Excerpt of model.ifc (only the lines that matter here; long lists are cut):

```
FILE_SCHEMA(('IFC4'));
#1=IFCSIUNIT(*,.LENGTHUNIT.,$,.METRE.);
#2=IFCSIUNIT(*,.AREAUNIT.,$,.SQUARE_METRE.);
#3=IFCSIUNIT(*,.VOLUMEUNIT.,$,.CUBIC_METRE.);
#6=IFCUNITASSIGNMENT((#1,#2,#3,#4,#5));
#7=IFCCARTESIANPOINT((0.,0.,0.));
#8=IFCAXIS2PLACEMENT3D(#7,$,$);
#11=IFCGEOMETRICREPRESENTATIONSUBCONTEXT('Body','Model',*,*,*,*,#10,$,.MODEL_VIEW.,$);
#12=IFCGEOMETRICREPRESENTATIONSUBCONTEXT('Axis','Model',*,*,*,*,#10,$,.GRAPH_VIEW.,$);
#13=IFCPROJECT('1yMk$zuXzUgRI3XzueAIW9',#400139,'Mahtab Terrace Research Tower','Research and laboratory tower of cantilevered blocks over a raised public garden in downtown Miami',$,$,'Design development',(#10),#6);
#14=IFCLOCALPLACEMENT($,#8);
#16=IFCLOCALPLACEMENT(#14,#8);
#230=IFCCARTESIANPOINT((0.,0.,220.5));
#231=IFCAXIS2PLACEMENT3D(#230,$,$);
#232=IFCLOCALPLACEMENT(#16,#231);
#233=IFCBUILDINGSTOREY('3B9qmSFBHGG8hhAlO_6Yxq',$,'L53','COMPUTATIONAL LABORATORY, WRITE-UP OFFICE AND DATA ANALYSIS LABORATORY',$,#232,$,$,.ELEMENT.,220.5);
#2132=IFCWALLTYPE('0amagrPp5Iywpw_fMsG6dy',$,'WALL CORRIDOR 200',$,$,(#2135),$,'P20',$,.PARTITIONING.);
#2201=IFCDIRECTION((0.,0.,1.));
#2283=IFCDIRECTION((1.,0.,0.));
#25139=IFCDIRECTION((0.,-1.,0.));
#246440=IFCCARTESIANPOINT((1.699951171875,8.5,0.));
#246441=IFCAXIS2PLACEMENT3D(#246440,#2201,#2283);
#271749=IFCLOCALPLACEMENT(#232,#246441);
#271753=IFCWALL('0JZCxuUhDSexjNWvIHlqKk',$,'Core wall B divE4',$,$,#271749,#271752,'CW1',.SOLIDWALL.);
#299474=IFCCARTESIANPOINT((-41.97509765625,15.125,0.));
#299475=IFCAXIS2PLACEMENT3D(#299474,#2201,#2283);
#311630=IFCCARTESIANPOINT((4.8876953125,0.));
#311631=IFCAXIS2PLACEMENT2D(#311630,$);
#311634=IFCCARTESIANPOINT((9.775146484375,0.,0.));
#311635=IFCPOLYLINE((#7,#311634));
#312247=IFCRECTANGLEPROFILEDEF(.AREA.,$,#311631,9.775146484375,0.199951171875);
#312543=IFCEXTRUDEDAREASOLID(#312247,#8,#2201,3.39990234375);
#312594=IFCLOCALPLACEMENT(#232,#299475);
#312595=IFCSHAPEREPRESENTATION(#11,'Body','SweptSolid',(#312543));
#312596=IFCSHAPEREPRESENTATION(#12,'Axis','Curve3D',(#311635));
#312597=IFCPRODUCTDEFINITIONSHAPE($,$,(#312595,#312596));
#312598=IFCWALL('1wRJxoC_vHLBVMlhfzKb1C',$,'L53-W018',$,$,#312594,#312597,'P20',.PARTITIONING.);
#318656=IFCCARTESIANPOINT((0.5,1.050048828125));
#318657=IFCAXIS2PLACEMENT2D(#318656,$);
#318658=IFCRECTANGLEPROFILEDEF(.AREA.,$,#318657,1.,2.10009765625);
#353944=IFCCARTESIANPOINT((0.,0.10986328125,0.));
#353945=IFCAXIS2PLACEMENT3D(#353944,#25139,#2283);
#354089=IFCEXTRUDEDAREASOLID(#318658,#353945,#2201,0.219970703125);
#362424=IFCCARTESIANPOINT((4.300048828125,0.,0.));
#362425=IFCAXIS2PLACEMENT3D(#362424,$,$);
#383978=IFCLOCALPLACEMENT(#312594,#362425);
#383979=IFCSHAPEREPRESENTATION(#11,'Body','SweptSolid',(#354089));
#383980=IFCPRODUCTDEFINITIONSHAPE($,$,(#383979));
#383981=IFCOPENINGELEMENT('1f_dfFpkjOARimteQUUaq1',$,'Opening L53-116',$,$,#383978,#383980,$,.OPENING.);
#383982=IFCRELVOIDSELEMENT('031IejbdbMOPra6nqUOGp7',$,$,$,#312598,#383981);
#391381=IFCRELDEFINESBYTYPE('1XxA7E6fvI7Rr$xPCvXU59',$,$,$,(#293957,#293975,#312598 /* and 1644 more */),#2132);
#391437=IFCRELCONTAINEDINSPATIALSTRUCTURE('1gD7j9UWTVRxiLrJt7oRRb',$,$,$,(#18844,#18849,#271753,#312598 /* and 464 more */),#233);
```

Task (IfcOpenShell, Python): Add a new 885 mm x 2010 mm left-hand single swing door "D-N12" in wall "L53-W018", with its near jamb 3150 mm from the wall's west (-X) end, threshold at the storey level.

```python
import numpy as np
import ifcopenshell
import ifcopenshell.api.feature
import ifcopenshell.api.geometry
import ifcopenshell.api.root
import ifcopenshell.api.spatial
import ifcopenshell.geom
import ifcopenshell.util.element
import ifcopenshell.util.placement
import ifcopenshell.util.representation
import ifcopenshell.util.shape
import ifcopenshell.util.unit

model = ifcopenshell.open("model.ifc")
unit_scale = ifcopenshell.util.unit.calculate_unit_scale(model)
settings = ifcopenshell.geom.settings()


def volume(element):
    """Net volume in cubic metres, openings subtracted."""
    shape = ifcopenshell.geom.create_shape(settings, element)
    return ifcopenshell.util.shape.get_volume(shape.geometry)


wall = model.by_guid("1wRJxoC_vHLBVMlhfzKb1C")
storey = ifcopenshell.util.element.get_container(wall, ifc_class="IfcBuildingStorey")
context = ifcopenshell.util.representation.get_context(model, "Model", "Body", "MODEL_VIEW")
before = volume(wall)

width, height, from_end, sill = 0.885, 2.01, 3.15, 0.0  # metres

# The wall runs along its own X axis, and the end named is its -X end.
wall_shape = ifcopenshell.geom.create_shape(settings, wall)
x, y, z = ifcopenshell.util.shape.get_vertices(wall_shape.geometry).T
start = x.min() + from_end
face, thickness = float(y.min()), float(y.max() - y.min())
wall_matrix = ifcopenshell.util.placement.get_local_placement(wall.ObjectPlacement)
level = ifcopenshell.util.placement.get_local_placement(storey.ObjectPlacement)[2, 3]


def in_wall(x, y):
    """Placement at x, y metres in the wall's axes, at sill height."""
    matrix = wall_matrix.copy()
    matrix[:, 3] = wall_matrix @ np.array([x / unit_scale, y / unit_scale, 0.0, 1.0])
    matrix[2, 3] = level + sill / unit_scale
    return matrix


# Opening: a box that overshoots both wall faces by 50 mm.
opening = ifcopenshell.api.root.create_entity(model, ifc_class="IfcOpeningElement", predefined_type="OPENING")
box = ifcopenshell.api.geometry.add_wall_representation(
    model, context=context, length=width, height=height, thickness=thickness + 0.1
)
ifcopenshell.api.geometry.assign_representation(model, product=opening, representation=box)
ifcopenshell.api.geometry.edit_object_placement(model, product=opening, matrix=in_wall(start, face - 0.05), is_si=False)
ifcopenshell.api.feature.add_feature(model, feature=opening, element=wall)

door = ifcopenshell.api.root.create_entity(model, ifc_class="IfcDoor", name="D-N12", predefined_type="DOOR")
door.OverallWidth, door.OverallHeight = width / unit_scale, height / unit_scale
door.OperationType = "SINGLE_SWING_LEFT"
body = ifcopenshell.api.geometry.add_door_representation(
    model,
    context=context,
    overall_width=door.OverallWidth,
    overall_height=door.OverallHeight,
    operation_type="SINGLE_SWING_LEFT",
    lining_properties={"LiningDepth": thickness / unit_scale, "ThresholdDepth": thickness / unit_scale},
)
ifcopenshell.api.geometry.assign_representation(model, product=door, representation=body)
ifcopenshell.api.spatial.assign_container(model, products=[door], relating_structure=storey)
ifcopenshell.api.feature.add_filling(model, opening=opening, element=door)

# The lining spans the wall, so the door starts at the wall face.
ifcopenshell.api.geometry.edit_object_placement(model, product=door, matrix=in_wall(start, face), is_si=False)

after = volume(wall)

print(f"wall volume {before:.3f} -> {after:.3f} m3")

model.write("model_rev.ifc")
```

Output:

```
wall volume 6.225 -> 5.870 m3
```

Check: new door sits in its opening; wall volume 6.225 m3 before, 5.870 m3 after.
